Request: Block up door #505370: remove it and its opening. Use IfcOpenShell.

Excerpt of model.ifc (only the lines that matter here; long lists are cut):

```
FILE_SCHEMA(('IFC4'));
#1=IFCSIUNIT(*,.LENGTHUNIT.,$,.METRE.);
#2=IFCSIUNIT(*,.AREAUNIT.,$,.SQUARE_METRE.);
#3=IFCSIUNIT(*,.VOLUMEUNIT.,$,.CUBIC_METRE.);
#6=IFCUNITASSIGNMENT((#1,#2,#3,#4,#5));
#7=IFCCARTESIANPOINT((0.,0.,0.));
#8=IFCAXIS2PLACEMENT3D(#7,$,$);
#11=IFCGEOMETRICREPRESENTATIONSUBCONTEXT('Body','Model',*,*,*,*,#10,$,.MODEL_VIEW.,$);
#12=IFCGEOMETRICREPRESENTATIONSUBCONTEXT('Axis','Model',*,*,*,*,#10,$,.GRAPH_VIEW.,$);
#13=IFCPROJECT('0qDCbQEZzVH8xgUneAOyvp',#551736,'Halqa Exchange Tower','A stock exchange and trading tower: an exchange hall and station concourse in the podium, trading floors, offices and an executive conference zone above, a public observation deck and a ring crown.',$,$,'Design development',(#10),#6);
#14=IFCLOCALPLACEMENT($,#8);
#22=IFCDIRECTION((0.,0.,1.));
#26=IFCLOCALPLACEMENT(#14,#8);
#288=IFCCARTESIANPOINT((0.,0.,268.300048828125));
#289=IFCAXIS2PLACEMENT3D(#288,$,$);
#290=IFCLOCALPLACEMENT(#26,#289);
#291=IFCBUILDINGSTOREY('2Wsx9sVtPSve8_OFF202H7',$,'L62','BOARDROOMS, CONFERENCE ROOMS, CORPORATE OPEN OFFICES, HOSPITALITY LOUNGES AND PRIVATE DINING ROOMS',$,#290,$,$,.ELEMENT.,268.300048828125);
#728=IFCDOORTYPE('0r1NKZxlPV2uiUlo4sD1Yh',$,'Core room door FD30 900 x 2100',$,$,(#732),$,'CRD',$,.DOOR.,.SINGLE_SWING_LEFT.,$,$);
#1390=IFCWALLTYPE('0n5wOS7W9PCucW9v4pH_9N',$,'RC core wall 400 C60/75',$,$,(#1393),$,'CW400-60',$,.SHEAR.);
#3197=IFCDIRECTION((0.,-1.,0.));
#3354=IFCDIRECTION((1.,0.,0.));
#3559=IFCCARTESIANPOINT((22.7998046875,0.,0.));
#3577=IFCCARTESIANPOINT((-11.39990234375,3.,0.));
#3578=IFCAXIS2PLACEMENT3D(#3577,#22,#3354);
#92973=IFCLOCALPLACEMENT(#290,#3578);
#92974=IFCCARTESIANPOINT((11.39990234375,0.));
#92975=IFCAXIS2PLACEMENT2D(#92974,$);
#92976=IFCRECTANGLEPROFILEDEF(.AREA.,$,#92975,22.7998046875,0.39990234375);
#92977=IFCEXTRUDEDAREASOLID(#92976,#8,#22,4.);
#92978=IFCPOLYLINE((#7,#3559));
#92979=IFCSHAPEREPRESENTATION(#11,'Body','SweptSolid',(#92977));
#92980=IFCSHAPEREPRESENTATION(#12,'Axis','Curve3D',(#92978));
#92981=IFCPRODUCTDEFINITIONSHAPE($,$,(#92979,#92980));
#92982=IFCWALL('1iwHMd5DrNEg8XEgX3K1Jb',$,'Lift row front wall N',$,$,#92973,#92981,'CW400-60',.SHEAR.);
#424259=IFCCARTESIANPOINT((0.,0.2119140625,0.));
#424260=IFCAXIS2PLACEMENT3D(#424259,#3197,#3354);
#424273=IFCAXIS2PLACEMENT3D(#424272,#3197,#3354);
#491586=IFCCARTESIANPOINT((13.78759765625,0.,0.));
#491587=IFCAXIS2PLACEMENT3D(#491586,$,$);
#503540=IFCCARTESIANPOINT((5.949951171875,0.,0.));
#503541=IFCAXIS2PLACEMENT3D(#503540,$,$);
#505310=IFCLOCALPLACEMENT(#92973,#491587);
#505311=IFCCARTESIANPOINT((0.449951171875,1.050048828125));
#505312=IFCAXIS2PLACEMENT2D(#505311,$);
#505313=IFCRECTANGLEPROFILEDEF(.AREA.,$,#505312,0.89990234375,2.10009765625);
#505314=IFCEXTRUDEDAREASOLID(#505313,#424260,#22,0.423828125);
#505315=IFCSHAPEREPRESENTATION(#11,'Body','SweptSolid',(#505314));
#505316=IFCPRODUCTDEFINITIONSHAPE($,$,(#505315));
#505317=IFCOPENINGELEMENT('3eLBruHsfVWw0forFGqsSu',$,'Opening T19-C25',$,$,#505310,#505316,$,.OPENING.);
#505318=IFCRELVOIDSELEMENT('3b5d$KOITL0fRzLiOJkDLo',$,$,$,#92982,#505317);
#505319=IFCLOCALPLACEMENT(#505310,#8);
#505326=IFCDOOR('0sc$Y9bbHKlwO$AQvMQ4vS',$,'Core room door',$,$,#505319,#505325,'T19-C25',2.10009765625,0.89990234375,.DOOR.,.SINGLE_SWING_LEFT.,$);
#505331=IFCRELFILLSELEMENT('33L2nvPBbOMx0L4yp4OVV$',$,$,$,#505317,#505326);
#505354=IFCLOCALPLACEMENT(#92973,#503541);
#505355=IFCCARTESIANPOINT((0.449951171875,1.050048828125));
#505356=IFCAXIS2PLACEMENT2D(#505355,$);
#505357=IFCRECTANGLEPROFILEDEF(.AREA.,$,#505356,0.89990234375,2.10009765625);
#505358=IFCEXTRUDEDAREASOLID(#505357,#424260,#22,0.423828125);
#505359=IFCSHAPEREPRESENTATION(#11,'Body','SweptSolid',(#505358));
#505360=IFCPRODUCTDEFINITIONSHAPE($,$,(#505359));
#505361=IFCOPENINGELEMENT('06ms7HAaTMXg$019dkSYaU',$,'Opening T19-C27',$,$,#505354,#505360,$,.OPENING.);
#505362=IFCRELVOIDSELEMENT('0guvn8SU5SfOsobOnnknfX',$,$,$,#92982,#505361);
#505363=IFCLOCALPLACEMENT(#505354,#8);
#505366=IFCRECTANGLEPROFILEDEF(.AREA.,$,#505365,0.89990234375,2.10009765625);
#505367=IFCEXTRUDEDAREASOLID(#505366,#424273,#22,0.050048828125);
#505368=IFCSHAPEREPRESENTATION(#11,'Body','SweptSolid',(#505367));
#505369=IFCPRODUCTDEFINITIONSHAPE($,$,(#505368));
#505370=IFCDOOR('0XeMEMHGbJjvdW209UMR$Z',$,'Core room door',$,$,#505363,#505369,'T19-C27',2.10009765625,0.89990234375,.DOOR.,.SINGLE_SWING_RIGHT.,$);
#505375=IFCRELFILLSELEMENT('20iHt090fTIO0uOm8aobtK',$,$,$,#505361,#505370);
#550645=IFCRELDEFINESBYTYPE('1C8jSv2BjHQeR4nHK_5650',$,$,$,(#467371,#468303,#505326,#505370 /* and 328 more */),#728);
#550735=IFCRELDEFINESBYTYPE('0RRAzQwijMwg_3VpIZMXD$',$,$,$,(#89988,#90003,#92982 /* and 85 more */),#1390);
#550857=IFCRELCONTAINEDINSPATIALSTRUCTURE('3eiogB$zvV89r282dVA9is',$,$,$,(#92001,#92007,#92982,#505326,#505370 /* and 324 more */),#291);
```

```python
import ifcopenshell
import ifcopenshell.api.feature
import ifcopenshell.api.root
import ifcopenshell.geom
import ifcopenshell.util.shape

model = ifcopenshell.open("model.ifc")
settings = ifcopenshell.geom.settings()


def volume(element):
    """Net volume in cubic metres, openings subtracted."""
    shape = ifcopenshell.geom.create_shape(settings, element)
    return ifcopenshell.util.shape.get_volume(shape.geometry)


door = model.by_id(505370)
opening = door.FillsVoids[0].RelatingOpeningElement
wall = opening.VoidsElements[0].RelatingBuildingElement
before = volume(wall)

ifcopenshell.api.root.remove_product(model, product=door)
ifcopenshell.api.feature.remove_feature(model, feature=opening)

after = volume(wall)

print(f"wall volume {before:.3f} -> {after:.3f} m3")

model.write("model_edited.ifc")
```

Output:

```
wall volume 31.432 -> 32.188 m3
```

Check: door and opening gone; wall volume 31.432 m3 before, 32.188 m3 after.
